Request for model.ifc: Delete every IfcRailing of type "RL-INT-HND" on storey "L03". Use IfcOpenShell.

First a look at what the model holds.

```python
import ifcopenshell
import ifcopenshell.util.element

model = ifcopenshell.open("model.ifc")
print(model.schema)
storey = next(s for s in model.by_type("IfcBuildingStorey") if s.Name == "L03")
railings = [e for e in ifcopenshell.util.element.get_decomposition(storey) if e.is_a("IfcRailing")]
seen = {}
for e in railings:
    element_type = ifcopenshell.util.element.get_type(e)
    name = element_type.Name if element_type not in (None, e) else None
    seen[name] = seen.get(name, 0) + 1
for name, count in sorted(seen.items(), key=str):
    print(count, "x", name)
```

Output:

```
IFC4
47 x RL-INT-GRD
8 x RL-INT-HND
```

```python
import ifcopenshell
import ifcopenshell.api.root
import ifcopenshell.util.element

model = ifcopenshell.open("model.ifc")

storey = next(s for s in model.by_type("IfcBuildingStorey") if s.Name == "L03")
railings = [e for e in ifcopenshell.util.element.get_decomposition(storey) if e.is_a("IfcRailing")]
targets = [e for e in railings if (t := ifcopenshell.util.element.get_type(e)) not in (None, e) and t.Name == "RL-INT-HND"]

for e in targets:
    ifcopenshell.api.root.remove_product(model, product=e)
print(len(targets), "removed")

model.write("model_updated.ifc")
```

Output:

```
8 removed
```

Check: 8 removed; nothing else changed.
